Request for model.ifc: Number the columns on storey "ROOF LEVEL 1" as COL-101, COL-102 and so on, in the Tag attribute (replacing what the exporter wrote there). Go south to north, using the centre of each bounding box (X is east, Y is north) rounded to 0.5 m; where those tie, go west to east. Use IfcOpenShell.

First a look at what the model holds.

```python
import ifcopenshell
import ifcopenshell.util.element
import ifcopenshell.util.placement

model = ifcopenshell.open("model.ifc")
print(model.schema)
storey = next(s for s in model.by_type("IfcBuildingStorey") if s.Name == "ROOF LEVEL 1")
columns = [e for e in ifcopenshell.util.element.get_decomposition(storey) if e.is_a("IfcColumn")]
for e in sorted(columns, key=lambda e: e.id()):
    origin = ifcopenshell.util.placement.get_local_placement(e.ObjectPlacement)[:3, 3]
    print(e.id(), e.Tag, e.Name, origin.round(2) + 0.0, sep=" | ")
```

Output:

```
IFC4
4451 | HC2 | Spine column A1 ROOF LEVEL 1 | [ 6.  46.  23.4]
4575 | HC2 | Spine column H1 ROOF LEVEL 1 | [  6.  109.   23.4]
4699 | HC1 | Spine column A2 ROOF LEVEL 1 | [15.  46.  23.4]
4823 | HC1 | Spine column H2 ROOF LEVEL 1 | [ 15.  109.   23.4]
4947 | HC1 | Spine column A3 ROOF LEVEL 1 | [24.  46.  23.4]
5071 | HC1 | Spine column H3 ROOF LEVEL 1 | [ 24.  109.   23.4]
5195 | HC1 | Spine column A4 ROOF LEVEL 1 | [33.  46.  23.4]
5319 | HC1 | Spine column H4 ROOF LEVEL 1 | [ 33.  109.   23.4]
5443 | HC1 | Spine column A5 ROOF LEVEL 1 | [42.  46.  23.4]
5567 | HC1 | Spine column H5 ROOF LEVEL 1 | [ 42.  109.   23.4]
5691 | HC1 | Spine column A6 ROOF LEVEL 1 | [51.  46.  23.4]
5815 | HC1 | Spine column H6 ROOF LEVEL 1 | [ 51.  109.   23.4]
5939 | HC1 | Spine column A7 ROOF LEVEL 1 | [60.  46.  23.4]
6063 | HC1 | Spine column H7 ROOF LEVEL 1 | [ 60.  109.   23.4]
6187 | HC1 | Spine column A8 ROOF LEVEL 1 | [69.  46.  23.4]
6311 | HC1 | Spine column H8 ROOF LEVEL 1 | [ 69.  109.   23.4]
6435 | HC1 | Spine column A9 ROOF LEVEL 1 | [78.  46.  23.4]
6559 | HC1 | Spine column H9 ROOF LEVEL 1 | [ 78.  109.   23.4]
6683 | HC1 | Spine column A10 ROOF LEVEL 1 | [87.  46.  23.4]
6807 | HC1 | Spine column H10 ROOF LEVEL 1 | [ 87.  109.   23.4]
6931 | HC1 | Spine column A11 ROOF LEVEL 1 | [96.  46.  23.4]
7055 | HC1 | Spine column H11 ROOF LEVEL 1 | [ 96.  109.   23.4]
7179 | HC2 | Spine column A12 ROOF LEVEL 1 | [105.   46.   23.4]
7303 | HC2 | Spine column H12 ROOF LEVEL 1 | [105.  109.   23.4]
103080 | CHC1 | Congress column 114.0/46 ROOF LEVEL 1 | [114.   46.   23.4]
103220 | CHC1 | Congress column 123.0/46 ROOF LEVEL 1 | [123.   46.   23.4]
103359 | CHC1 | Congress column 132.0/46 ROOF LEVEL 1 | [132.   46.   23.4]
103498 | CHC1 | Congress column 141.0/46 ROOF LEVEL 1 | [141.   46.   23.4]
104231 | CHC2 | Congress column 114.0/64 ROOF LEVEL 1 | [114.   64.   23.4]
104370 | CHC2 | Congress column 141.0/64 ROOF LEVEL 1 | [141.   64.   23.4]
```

```python
import ifcopenshell
import ifcopenshell.geom
import ifcopenshell.util.element
import ifcopenshell.util.shape

model = ifcopenshell.open("model.ifc")
settings = ifcopenshell.geom.settings()
settings.set("use-world-coords", True)


def centre(element):
    shape = ifcopenshell.geom.create_shape(settings, element)
    return ifcopenshell.util.shape.get_bbox_centroid(shape.geometry)


storey = next(s for s in model.by_type("IfcBuildingStorey") if s.Name == "ROOF LEVEL 1")
columns = [e for e in ifcopenshell.util.element.get_decomposition(storey) if e.is_a("IfcColumn")]

# Insertion points can sit at a corner or the storey origin, so sort by the geometry (in metres).
centres = {e: centre(e) for e in columns}
columns.sort(key=lambda e: (round(centres[e][1] / 0.5), centres[e][0]))

for i, e in enumerate(columns, start=1):
    number = f"COL-1{i:02d}"
    e.Tag = number
    print(e.id(), number)

model.write("model-out.ifc")
```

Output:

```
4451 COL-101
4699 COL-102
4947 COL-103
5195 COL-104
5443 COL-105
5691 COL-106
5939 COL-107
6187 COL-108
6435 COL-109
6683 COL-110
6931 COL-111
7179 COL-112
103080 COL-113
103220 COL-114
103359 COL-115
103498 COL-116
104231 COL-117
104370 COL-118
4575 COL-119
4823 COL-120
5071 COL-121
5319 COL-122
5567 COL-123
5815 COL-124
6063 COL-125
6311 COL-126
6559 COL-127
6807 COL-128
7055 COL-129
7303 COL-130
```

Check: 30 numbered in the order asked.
